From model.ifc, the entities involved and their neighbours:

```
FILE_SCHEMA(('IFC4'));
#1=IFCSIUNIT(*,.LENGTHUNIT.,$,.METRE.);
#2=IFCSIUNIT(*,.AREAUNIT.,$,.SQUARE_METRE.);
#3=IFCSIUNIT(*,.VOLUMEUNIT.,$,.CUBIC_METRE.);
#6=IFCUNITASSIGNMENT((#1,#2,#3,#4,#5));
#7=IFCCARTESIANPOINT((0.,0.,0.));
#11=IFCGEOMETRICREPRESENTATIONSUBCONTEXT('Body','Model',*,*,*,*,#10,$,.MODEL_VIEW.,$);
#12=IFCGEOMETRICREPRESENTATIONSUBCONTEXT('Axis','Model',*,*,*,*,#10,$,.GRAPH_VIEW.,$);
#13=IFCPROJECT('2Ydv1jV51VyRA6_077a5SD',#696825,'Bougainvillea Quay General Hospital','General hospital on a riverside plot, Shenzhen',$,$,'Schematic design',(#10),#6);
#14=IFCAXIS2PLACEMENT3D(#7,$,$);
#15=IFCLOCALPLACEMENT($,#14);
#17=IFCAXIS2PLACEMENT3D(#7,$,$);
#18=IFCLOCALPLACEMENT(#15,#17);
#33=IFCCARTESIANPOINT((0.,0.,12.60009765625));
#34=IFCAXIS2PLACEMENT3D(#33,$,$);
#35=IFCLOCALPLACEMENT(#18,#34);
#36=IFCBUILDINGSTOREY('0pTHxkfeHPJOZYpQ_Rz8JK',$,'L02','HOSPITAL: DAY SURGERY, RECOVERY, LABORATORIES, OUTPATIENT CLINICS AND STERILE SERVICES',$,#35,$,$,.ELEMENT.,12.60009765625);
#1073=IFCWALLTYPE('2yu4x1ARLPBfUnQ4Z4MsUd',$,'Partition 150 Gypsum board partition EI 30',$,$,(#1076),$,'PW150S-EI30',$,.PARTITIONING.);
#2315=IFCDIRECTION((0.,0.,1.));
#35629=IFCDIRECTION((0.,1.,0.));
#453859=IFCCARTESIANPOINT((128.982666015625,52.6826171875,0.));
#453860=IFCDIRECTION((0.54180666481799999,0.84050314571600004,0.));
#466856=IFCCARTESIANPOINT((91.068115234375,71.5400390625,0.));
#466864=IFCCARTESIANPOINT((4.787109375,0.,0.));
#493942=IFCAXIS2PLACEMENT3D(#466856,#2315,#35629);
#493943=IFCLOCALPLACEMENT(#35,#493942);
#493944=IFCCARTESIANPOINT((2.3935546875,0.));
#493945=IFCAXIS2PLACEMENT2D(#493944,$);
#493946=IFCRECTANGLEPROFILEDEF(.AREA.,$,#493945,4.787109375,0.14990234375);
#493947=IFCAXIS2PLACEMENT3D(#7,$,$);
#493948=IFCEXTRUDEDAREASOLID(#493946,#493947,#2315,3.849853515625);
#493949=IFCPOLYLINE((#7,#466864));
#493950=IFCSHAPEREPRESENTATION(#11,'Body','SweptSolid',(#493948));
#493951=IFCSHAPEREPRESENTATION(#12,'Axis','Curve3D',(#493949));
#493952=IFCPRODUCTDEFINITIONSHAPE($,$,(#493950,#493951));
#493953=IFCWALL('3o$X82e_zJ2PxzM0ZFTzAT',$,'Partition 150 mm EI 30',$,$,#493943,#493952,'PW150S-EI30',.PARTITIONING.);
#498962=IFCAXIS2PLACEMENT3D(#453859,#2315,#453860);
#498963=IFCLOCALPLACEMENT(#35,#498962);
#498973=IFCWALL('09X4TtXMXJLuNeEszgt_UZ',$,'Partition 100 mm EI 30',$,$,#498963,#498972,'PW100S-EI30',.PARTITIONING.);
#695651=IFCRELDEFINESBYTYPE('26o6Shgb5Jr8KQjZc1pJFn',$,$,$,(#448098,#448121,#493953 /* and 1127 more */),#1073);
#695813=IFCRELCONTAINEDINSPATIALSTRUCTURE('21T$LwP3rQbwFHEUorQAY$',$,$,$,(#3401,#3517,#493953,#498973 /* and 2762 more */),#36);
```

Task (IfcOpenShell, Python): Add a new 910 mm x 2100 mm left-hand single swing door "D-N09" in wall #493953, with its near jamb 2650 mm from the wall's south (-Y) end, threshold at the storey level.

```python
import numpy as np
import ifcopenshell
import ifcopenshell.api.feature
import ifcopenshell.api.geometry
import ifcopenshell.api.root
import ifcopenshell.api.spatial
import ifcopenshell.geom
import ifcopenshell.util.element
import ifcopenshell.util.placement
import ifcopenshell.util.representation
import ifcopenshell.util.shape
import ifcopenshell.util.unit

model = ifcopenshell.open("model.ifc")
unit_scale = ifcopenshell.util.unit.calculate_unit_scale(model)
settings = ifcopenshell.geom.settings()


def volume(element):
    """Net volume in cubic metres, openings subtracted."""
    shape = ifcopenshell.geom.create_shape(settings, element)
    return ifcopenshell.util.shape.get_volume(shape.geometry)


wall = model.by_id(493953)
storey = ifcopenshell.util.element.get_container(wall, ifc_class="IfcBuildingStorey")
context = ifcopenshell.util.representation.get_context(model, "Model", "Body", "MODEL_VIEW")
before = volume(wall)

width, height, from_end, sill = 0.91, 2.1, 2.65, 0.0  # metres

# The wall runs along its own X axis, and the end named is its -X end.
wall_shape = ifcopenshell.geom.create_shape(settings, wall)
x, y, z = ifcopenshell.util.shape.get_vertices(wall_shape.geometry).T
start = x.min() + from_end
face, thickness = float(y.min()), float(y.max() - y.min())
wall_matrix = ifcopenshell.util.placement.get_local_placement(wall.ObjectPlacement)
level = ifcopenshell.util.placement.get_local_placement(storey.ObjectPlacement)[2, 3]


def in_wall(x, y):
    """Placement at x, y metres in the wall's axes, at sill height."""
    matrix = wall_matrix.copy()
    matrix[:, 3] = wall_matrix @ np.array([x / unit_scale, y / unit_scale, 0.0, 1.0])
    matrix[2, 3] = level + sill / unit_scale
    return matrix


# Opening: a box that overshoots both wall faces by 50 mm.
opening = ifcopenshell.api.root.create_entity(model, ifc_class="IfcOpeningElement", predefined_type="OPENING")
box = ifcopenshell.api.geometry.add_wall_representation(
    model, context=context, length=width, height=height, thickness=thickness + 0.1
)
ifcopenshell.api.geometry.assign_representation(model, product=opening, representation=box)
ifcopenshell.api.geometry.edit_object_placement(model, product=opening, matrix=in_wall(start, face - 0.05), is_si=False)
ifcopenshell.api.feature.add_feature(model, feature=opening, element=wall)

door = ifcopenshell.api.root.create_entity(model, ifc_class="IfcDoor", name="D-N09", predefined_type="DOOR")
door.OverallWidth, door.OverallHeight = width / unit_scale, height / unit_scale
door.OperationType = "SINGLE_SWING_LEFT"
body = ifcopenshell.api.geometry.add_door_representation(
    model,
    context=context,
    overall_width=door.OverallWidth,
    overall_height=door.OverallHeight,
    operation_type="SINGLE_SWING_LEFT",
    lining_properties={"LiningDepth": thickness / unit_scale, "ThresholdDepth": thickness / unit_scale},
)
ifcopenshell.api.geometry.assign_representation(model, product=door, representation=body)
ifcopenshell.api.spatial.assign_container(model, products=[door], relating_structure=storey)
ifcopenshell.api.feature.add_filling(model, opening=opening, element=door)

# The lining spans the wall, so the door starts at the wall face.
ifcopenshell.api.geometry.edit_object_placement(model, product=door, matrix=in_wall(start, face), is_si=False)

after = volume(wall)

print(f"wall volume {before:.3f} -> {after:.3f} m3")

model.write("model_rev.ifc")
```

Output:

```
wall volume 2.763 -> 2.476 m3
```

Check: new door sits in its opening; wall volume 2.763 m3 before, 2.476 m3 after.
